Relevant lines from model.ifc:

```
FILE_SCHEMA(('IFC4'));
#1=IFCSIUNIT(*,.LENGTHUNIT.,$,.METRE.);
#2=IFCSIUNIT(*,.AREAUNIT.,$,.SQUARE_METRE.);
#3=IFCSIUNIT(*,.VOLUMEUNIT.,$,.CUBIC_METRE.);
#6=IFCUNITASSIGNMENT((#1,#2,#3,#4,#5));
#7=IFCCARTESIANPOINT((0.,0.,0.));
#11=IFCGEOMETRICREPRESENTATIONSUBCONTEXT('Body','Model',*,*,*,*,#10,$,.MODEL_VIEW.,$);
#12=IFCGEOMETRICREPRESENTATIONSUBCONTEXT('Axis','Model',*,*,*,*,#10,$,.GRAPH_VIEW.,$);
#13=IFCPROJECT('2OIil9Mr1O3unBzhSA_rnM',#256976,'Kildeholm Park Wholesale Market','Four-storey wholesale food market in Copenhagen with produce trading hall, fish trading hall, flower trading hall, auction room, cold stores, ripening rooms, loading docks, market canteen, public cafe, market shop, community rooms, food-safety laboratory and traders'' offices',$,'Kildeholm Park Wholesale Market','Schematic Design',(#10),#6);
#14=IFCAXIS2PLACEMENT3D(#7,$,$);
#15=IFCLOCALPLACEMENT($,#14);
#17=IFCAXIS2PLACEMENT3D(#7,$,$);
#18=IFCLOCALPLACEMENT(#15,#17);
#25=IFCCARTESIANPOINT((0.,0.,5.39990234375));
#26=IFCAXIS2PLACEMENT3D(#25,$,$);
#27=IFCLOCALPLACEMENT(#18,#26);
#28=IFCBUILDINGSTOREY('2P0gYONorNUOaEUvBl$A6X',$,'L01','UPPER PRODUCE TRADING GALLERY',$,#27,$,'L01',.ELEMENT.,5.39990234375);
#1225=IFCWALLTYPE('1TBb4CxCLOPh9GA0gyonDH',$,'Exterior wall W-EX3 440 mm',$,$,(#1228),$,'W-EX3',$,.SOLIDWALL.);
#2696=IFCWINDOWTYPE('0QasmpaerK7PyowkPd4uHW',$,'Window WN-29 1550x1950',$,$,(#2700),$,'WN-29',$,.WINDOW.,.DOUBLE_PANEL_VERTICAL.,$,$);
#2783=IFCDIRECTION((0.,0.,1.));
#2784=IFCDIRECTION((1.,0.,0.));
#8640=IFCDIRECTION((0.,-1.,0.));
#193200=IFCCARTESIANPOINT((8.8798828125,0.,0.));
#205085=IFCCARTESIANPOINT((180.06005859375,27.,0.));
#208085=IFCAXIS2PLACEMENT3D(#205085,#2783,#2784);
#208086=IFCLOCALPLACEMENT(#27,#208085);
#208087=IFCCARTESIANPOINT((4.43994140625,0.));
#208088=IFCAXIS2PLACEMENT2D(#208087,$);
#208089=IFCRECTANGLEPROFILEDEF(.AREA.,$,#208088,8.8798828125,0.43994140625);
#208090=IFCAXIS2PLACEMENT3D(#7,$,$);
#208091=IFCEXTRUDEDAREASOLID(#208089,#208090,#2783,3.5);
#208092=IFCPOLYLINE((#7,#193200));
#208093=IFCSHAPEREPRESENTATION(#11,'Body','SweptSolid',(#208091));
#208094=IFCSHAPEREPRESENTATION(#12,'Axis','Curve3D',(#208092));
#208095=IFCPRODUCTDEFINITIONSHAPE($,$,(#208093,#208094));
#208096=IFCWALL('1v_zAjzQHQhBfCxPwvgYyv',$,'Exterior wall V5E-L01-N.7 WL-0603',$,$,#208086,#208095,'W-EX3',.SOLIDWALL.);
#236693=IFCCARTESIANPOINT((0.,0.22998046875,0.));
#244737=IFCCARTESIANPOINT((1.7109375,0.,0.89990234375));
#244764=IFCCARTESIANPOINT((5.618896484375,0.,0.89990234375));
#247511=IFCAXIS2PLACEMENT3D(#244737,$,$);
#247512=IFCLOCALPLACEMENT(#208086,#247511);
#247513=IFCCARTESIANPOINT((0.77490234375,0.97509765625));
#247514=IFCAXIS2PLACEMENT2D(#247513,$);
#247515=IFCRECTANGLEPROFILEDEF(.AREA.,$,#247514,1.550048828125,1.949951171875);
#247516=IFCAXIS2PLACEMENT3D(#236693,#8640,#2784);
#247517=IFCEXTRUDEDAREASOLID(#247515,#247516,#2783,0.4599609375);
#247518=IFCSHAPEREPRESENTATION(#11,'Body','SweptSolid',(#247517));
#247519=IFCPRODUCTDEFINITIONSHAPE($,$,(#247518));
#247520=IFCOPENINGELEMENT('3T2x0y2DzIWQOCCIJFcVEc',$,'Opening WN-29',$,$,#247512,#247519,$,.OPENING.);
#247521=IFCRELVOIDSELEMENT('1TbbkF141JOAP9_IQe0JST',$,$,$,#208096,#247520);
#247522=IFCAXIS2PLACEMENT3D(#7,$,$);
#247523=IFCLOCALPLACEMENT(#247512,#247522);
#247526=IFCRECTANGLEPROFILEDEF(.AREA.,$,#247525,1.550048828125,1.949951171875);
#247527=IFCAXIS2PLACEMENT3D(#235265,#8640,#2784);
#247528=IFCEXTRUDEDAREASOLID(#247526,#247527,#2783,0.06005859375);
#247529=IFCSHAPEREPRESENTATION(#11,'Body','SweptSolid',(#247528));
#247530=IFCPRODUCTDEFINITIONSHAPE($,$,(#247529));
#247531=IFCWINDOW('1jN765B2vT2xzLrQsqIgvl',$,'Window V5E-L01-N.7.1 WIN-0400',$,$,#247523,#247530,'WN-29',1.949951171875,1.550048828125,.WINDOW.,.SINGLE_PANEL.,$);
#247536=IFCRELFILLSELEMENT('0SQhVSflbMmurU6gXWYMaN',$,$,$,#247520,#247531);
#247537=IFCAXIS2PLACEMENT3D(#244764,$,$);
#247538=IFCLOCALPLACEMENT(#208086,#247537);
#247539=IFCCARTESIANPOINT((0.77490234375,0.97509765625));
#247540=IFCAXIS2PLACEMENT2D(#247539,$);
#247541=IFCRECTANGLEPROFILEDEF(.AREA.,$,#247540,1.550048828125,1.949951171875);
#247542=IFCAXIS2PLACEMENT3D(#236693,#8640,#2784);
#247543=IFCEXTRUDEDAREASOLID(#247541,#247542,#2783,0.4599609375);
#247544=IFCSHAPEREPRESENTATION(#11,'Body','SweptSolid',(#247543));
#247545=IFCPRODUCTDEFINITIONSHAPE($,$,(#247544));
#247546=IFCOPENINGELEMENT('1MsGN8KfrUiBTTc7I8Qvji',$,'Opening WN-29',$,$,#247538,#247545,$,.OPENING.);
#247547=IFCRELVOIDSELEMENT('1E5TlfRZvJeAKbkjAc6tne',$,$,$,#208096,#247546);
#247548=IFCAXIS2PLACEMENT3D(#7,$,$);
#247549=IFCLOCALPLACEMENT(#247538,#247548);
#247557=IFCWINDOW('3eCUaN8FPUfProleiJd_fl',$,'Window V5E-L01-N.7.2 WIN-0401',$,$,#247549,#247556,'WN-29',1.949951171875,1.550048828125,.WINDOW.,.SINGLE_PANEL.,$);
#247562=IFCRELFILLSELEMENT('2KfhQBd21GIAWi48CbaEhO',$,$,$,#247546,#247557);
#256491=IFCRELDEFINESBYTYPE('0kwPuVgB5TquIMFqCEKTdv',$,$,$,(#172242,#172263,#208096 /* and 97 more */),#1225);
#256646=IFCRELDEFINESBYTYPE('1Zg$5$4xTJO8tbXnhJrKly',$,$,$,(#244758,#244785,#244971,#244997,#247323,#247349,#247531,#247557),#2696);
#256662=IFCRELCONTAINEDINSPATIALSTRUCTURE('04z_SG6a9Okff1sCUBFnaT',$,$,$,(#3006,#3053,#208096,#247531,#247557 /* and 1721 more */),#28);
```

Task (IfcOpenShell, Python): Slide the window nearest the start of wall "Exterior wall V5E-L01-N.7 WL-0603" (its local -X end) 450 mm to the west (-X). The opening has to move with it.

```python
import ifcopenshell
import ifcopenshell.api.geometry
import ifcopenshell.util.placement

model = ifcopenshell.open("model.ifc")

window = model.by_guid("1jN765B2vT2xzLrQsqIgvl")
opening = window.FillsVoids[0].RelatingOpeningElement
wall = opening.VoidsElements[0].RelatingBuildingElement

wall_matrix = ifcopenshell.util.placement.get_local_placement(wall.ObjectPlacement)
shift = wall_matrix[:3, 0] * -0.45
before = ifcopenshell.util.placement.get_local_placement(window.ObjectPlacement)[:3, 3].copy()

# The window is placed relative to its opening, so it follows when the opening moves.
matrix = ifcopenshell.util.placement.get_local_placement(opening.ObjectPlacement)
matrix[:3, 3] += shift
ifcopenshell.api.geometry.edit_object_placement(
    model, product=opening, matrix=matrix, is_si=False, should_transform_children=True
)

after = ifcopenshell.util.placement.get_local_placement(window.ObjectPlacement)[:3, 3]
print("window moved by", (after - before).round(3) + 0.0)

model.write("model_v2.ifc")
```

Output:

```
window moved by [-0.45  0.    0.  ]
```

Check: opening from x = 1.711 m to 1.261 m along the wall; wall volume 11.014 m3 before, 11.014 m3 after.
